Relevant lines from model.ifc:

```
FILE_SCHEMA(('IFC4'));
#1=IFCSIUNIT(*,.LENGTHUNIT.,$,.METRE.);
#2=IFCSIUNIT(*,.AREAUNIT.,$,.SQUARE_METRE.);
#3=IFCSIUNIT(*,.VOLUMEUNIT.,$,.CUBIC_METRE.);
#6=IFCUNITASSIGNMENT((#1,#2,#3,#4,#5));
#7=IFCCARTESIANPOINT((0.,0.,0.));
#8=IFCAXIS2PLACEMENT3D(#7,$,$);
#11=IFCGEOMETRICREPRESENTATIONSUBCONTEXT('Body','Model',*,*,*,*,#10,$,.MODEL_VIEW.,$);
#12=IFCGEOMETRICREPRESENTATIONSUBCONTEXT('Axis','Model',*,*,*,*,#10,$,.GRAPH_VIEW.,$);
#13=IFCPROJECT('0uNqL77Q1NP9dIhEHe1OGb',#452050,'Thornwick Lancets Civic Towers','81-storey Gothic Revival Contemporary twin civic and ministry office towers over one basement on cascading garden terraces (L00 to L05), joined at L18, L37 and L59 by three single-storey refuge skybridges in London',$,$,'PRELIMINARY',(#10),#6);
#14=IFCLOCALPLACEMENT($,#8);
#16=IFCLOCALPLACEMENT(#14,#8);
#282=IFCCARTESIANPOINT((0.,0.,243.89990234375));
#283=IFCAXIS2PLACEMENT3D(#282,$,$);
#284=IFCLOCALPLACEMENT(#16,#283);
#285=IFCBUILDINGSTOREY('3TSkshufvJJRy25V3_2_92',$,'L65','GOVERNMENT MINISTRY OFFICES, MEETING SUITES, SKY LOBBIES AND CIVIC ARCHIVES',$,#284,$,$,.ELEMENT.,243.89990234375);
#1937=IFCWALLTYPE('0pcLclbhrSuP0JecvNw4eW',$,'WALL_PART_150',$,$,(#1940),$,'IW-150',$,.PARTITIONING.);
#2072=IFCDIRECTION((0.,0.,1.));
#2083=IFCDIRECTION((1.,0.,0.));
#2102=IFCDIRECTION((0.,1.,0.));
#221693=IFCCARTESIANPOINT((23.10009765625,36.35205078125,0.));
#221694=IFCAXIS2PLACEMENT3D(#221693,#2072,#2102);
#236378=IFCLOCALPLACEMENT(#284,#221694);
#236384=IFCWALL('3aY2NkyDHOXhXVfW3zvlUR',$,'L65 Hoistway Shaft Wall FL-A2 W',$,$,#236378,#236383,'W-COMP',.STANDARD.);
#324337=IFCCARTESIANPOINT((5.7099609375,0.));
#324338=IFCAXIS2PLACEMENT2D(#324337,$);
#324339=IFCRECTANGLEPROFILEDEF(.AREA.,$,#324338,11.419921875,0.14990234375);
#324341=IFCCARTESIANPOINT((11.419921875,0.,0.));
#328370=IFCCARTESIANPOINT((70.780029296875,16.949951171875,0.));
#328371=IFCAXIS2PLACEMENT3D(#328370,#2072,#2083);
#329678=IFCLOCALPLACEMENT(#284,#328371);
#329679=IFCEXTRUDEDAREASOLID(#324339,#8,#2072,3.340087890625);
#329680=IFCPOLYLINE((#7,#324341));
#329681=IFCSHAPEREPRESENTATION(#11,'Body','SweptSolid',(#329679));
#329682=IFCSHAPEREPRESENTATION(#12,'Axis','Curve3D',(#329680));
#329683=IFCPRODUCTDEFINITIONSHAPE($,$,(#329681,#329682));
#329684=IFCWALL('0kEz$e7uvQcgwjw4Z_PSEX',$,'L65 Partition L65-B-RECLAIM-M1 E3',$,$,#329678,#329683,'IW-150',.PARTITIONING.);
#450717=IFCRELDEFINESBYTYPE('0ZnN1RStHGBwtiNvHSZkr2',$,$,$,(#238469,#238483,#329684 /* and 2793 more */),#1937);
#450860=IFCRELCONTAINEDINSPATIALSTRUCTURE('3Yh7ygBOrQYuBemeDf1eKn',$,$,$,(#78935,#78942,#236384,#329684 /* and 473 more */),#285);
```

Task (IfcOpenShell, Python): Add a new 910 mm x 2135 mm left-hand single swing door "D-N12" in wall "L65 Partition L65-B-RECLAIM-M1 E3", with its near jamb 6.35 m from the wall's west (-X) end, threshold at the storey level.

```python
import numpy as np
import ifcopenshell
import ifcopenshell.api.feature
import ifcopenshell.api.geometry
import ifcopenshell.api.root
import ifcopenshell.api.spatial
import ifcopenshell.geom
import ifcopenshell.util.element
import ifcopenshell.util.placement
import ifcopenshell.util.representation
import ifcopenshell.util.shape
import ifcopenshell.util.unit

model = ifcopenshell.open("model.ifc")
unit_scale = ifcopenshell.util.unit.calculate_unit_scale(model)
settings = ifcopenshell.geom.settings()


def volume(element):
    """Net volume in cubic metres, openings subtracted."""
    shape = ifcopenshell.geom.create_shape(settings, element)
    return ifcopenshell.util.shape.get_volume(shape.geometry)


wall = model.by_id(329684)
storey = ifcopenshell.util.element.get_container(wall, ifc_class="IfcBuildingStorey")
context = ifcopenshell.util.representation.get_context(model, "Model", "Body", "MODEL_VIEW")
before = volume(wall)

width, height, from_end, sill = 0.91, 2.135, 6.35, 0.0  # metres

# The wall runs along its own X axis, and the end named is its -X end.
wall_shape = ifcopenshell.geom.create_shape(settings, wall)
x, y, z = ifcopenshell.util.shape.get_vertices(wall_shape.geometry).T
start = x.min() + from_end
face, thickness = float(y.min()), float(y.max() - y.min())
wall_matrix = ifcopenshell.util.placement.get_local_placement(wall.ObjectPlacement)
level = ifcopenshell.util.placement.get_local_placement(storey.ObjectPlacement)[2, 3]


def in_wall(x, y):
    """Placement at x, y metres in the wall's axes, at sill height."""
    matrix = wall_matrix.copy()
    matrix[:, 3] = wall_matrix @ np.array([x / unit_scale, y / unit_scale, 0.0, 1.0])
    matrix[2, 3] = level + sill / unit_scale
    return matrix


# Opening: a box that overshoots both wall faces by 50 mm.
opening = ifcopenshell.api.root.create_entity(model, ifc_class="IfcOpeningElement", predefined_type="OPENING")
box = ifcopenshell.api.geometry.add_wall_representation(
    model, context=context, length=width, height=height, thickness=thickness + 0.1
)
ifcopenshell.api.geometry.assign_representation(model, product=opening, representation=box)
ifcopenshell.api.geometry.edit_object_placement(model, product=opening, matrix=in_wall(start, face - 0.05), is_si=False)
ifcopenshell.api.feature.add_feature(model, feature=opening, element=wall)

door = ifcopenshell.api.root.create_entity(model, ifc_class="IfcDoor", name="D-N12", predefined_type="DOOR")
door.OverallWidth, door.OverallHeight = width / unit_scale, height / unit_scale
door.OperationType = "SINGLE_SWING_LEFT"
body = ifcopenshell.api.geometry.add_door_representation(
    model,
    context=context,
    overall_width=door.OverallWidth,
    overall_height=door.OverallHeight,
    operation_type="SINGLE_SWING_LEFT",
    lining_properties={"LiningDepth": thickness / unit_scale, "ThresholdDepth": thickness / unit_scale},
)
ifcopenshell.api.geometry.assign_representation(model, product=door, representation=body)
ifcopenshell.api.spatial.assign_container(model, products=[door], relating_structure=storey)
ifcopenshell.api.feature.add_filling(model, opening=opening, element=door)

# The lining spans the wall, so the door starts at the wall face.
ifcopenshell.api.geometry.edit_object_placement(model, product=door, matrix=in_wall(start, face), is_si=False)

after = volume(wall)

print(f"wall volume {before:.3f} -> {after:.3f} m3")

model.write("model_updated.ifc")
```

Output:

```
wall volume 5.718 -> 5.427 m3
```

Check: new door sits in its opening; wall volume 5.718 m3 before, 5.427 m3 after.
